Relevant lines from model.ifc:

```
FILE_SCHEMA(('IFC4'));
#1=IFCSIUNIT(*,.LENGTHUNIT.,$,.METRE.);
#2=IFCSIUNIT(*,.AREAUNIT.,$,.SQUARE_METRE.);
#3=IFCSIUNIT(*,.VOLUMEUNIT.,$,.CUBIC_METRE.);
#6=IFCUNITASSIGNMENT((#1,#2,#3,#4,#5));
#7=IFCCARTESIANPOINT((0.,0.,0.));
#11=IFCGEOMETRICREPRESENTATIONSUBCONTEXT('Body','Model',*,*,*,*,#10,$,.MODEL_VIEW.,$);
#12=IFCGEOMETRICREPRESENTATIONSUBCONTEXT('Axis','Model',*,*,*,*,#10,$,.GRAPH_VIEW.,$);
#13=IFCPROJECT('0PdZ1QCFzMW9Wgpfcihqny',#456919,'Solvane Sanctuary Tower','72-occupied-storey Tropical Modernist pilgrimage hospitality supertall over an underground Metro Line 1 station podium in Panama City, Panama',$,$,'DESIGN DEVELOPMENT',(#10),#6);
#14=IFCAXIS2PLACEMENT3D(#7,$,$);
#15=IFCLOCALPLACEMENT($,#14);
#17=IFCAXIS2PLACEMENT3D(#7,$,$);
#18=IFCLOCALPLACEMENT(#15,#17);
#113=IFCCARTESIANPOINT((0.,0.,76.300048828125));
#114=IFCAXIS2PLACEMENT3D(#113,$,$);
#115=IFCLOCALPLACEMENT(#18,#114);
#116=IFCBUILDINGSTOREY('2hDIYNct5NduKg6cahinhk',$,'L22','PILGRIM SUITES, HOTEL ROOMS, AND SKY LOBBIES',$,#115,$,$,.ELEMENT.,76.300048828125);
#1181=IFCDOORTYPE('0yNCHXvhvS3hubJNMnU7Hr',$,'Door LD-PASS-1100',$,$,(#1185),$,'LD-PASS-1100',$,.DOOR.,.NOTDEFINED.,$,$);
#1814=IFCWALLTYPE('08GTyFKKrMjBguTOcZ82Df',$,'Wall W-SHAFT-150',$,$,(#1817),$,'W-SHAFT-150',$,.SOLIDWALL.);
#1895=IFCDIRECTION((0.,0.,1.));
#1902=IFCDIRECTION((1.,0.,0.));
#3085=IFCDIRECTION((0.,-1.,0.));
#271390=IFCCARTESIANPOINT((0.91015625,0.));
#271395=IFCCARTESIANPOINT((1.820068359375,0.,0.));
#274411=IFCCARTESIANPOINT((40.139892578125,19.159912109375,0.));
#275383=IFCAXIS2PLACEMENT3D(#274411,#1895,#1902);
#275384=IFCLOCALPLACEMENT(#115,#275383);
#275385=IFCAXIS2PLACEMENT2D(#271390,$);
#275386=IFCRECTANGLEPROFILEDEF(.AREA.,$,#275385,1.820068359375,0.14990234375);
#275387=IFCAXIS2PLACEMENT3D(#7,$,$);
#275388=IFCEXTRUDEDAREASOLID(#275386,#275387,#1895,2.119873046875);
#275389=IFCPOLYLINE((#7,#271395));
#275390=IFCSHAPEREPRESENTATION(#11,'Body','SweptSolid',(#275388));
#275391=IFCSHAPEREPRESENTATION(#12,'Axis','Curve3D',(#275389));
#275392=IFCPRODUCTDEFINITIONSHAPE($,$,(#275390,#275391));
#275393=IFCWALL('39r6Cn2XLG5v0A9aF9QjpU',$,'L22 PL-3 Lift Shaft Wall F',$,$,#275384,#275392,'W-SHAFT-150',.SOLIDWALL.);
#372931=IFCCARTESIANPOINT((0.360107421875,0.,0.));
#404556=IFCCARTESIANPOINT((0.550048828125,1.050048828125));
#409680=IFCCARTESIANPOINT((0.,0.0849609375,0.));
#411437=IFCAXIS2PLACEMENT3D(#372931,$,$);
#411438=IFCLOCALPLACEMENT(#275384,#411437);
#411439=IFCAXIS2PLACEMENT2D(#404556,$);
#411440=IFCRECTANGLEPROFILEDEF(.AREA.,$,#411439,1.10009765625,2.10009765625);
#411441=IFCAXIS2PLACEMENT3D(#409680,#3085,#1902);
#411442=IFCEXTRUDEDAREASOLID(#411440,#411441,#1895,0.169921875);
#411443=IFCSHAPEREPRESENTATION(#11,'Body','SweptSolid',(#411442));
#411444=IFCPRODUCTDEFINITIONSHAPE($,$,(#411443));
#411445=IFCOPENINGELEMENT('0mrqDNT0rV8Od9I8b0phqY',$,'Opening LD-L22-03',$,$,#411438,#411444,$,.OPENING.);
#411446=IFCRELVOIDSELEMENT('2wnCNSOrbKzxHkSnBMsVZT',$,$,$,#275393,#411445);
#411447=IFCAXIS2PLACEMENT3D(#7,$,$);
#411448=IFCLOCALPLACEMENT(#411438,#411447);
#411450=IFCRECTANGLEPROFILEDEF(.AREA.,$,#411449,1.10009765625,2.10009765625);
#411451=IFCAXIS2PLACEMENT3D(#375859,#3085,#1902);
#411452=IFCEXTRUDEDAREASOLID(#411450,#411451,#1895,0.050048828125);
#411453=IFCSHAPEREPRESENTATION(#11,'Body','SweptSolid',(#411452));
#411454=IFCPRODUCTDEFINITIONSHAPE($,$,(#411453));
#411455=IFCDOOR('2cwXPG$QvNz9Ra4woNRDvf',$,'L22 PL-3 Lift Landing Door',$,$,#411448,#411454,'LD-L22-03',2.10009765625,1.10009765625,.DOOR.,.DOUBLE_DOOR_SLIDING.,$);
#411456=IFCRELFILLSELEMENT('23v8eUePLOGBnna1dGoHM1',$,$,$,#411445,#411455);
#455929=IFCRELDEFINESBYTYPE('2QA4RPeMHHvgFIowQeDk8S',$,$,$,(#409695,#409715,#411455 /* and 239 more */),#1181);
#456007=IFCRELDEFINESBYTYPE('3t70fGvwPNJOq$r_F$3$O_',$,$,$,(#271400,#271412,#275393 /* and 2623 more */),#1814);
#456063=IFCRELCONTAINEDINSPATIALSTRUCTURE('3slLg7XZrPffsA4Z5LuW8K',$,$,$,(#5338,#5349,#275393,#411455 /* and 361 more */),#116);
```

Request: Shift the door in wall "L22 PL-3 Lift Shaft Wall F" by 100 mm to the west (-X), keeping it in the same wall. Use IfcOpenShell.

```python
import ifcopenshell
import ifcopenshell.api.geometry
import ifcopenshell.util.placement

model = ifcopenshell.open("model.ifc")

door = model.by_id(411455)
opening = door.FillsVoids[0].RelatingOpeningElement
wall = opening.VoidsElements[0].RelatingBuildingElement

wall_matrix = ifcopenshell.util.placement.get_local_placement(wall.ObjectPlacement)
shift = wall_matrix[:3, 0] * -0.1
before = ifcopenshell.util.placement.get_local_placement(door.ObjectPlacement)[:3, 3].copy()

# The door is placed relative to its opening, so it follows when the opening moves.
matrix = ifcopenshell.util.placement.get_local_placement(opening.ObjectPlacement)
matrix[:3, 3] += shift
ifcopenshell.api.geometry.edit_object_placement(
    model, product=opening, matrix=matrix, is_si=False, should_transform_children=True
)

after = ifcopenshell.util.placement.get_local_placement(door.ObjectPlacement)[:3, 3]
print("door moved by", (after - before).round(3) + 0.0)

model.write("model_updated.ifc")
```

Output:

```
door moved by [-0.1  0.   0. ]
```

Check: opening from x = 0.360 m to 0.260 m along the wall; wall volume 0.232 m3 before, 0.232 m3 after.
